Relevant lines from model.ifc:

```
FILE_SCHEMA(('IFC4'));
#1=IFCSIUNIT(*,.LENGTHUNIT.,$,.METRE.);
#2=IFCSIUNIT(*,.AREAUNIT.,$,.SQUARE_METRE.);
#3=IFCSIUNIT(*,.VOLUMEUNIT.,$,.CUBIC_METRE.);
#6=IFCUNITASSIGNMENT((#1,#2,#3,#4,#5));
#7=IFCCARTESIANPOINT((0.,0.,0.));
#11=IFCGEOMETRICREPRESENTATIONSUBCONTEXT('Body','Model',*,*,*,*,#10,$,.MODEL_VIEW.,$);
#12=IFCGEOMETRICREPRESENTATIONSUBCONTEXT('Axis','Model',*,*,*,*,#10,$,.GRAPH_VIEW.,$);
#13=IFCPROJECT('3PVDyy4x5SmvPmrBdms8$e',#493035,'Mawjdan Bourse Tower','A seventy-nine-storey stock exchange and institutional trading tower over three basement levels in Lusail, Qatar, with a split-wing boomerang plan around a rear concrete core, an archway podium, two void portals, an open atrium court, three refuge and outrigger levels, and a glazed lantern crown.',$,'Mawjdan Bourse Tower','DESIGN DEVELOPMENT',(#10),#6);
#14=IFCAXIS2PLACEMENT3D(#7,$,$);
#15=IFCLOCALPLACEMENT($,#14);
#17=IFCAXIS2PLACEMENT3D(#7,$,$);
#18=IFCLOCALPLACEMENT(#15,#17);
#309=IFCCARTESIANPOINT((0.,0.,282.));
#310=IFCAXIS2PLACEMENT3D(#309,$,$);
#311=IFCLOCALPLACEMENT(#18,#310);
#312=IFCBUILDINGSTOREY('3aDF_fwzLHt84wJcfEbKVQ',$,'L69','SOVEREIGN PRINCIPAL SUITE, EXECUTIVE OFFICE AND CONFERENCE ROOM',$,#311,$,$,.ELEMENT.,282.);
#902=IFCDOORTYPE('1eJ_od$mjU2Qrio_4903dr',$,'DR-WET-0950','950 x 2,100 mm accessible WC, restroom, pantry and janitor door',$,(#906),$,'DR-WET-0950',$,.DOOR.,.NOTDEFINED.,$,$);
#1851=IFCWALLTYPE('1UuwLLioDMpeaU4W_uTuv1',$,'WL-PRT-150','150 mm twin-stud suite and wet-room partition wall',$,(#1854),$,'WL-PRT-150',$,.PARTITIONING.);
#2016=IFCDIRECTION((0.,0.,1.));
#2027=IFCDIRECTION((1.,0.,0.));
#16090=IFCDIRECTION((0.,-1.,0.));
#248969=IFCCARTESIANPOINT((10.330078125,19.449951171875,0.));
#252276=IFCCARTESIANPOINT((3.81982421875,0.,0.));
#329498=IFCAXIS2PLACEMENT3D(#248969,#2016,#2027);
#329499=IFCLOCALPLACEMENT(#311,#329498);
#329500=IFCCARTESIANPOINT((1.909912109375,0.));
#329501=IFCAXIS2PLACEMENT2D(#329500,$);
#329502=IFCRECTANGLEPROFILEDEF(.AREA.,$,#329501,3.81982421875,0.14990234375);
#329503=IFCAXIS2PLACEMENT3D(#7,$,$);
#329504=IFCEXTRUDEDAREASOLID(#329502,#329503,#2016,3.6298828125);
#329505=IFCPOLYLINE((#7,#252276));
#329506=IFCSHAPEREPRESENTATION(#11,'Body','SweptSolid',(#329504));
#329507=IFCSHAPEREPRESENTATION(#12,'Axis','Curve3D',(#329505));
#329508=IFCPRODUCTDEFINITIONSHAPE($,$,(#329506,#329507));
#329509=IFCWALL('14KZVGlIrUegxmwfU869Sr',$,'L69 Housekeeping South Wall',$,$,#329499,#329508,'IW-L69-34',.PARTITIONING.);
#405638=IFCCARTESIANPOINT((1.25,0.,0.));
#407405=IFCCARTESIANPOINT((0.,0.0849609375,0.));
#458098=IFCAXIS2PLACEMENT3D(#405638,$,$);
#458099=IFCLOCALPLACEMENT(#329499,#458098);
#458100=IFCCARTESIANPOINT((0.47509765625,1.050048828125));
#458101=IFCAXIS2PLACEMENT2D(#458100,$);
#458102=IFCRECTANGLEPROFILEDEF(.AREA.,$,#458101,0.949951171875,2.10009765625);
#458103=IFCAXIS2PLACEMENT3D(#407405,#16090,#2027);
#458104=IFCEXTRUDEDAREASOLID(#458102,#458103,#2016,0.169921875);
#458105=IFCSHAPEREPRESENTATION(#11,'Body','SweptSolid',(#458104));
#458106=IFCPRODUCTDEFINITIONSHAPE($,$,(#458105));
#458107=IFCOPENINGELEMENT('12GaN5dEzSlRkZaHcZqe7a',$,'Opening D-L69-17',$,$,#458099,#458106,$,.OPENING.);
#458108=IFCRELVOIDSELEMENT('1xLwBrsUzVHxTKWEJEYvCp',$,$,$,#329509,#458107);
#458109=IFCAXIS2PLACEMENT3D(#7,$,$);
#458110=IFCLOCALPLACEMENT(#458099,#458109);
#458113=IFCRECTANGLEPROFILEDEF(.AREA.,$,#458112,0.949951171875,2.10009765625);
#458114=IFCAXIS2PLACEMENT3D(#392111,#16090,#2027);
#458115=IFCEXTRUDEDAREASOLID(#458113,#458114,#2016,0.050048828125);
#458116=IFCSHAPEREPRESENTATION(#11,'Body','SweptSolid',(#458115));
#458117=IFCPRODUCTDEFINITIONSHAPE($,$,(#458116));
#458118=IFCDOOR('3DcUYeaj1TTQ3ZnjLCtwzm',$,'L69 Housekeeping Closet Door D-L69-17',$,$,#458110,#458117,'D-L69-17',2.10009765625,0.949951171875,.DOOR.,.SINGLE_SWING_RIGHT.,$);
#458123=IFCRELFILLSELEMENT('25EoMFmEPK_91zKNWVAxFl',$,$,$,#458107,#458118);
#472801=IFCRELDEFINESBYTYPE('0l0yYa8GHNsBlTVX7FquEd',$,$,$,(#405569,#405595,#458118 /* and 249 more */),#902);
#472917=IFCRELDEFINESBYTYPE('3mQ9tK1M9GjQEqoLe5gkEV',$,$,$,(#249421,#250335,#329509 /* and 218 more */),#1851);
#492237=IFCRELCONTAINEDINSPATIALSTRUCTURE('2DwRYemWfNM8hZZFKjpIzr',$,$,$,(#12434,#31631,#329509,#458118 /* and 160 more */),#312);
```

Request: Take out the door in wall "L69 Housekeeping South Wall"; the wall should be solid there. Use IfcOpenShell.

```python
import ifcopenshell
import ifcopenshell.api.feature
import ifcopenshell.api.root
import ifcopenshell.geom
import ifcopenshell.util.shape

model = ifcopenshell.open("model.ifc")
settings = ifcopenshell.geom.settings()


def volume(element):
    """Net volume in cubic metres, openings subtracted."""
    shape = ifcopenshell.geom.create_shape(settings, element)
    return ifcopenshell.util.shape.get_volume(shape.geometry)


door = model.by_guid("3DcUYeaj1TTQ3ZnjLCtwzm")
opening = door.FillsVoids[0].RelatingOpeningElement
wall = opening.VoidsElements[0].RelatingBuildingElement
before = volume(wall)

ifcopenshell.api.root.remove_product(model, product=door)
ifcopenshell.api.feature.remove_feature(model, feature=opening)

after = volume(wall)

print(f"wall volume {before:.3f} -> {after:.3f} m3")

model.write("model_v2.ifc")
```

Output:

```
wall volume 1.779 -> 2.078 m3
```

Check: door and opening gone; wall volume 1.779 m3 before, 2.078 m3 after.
